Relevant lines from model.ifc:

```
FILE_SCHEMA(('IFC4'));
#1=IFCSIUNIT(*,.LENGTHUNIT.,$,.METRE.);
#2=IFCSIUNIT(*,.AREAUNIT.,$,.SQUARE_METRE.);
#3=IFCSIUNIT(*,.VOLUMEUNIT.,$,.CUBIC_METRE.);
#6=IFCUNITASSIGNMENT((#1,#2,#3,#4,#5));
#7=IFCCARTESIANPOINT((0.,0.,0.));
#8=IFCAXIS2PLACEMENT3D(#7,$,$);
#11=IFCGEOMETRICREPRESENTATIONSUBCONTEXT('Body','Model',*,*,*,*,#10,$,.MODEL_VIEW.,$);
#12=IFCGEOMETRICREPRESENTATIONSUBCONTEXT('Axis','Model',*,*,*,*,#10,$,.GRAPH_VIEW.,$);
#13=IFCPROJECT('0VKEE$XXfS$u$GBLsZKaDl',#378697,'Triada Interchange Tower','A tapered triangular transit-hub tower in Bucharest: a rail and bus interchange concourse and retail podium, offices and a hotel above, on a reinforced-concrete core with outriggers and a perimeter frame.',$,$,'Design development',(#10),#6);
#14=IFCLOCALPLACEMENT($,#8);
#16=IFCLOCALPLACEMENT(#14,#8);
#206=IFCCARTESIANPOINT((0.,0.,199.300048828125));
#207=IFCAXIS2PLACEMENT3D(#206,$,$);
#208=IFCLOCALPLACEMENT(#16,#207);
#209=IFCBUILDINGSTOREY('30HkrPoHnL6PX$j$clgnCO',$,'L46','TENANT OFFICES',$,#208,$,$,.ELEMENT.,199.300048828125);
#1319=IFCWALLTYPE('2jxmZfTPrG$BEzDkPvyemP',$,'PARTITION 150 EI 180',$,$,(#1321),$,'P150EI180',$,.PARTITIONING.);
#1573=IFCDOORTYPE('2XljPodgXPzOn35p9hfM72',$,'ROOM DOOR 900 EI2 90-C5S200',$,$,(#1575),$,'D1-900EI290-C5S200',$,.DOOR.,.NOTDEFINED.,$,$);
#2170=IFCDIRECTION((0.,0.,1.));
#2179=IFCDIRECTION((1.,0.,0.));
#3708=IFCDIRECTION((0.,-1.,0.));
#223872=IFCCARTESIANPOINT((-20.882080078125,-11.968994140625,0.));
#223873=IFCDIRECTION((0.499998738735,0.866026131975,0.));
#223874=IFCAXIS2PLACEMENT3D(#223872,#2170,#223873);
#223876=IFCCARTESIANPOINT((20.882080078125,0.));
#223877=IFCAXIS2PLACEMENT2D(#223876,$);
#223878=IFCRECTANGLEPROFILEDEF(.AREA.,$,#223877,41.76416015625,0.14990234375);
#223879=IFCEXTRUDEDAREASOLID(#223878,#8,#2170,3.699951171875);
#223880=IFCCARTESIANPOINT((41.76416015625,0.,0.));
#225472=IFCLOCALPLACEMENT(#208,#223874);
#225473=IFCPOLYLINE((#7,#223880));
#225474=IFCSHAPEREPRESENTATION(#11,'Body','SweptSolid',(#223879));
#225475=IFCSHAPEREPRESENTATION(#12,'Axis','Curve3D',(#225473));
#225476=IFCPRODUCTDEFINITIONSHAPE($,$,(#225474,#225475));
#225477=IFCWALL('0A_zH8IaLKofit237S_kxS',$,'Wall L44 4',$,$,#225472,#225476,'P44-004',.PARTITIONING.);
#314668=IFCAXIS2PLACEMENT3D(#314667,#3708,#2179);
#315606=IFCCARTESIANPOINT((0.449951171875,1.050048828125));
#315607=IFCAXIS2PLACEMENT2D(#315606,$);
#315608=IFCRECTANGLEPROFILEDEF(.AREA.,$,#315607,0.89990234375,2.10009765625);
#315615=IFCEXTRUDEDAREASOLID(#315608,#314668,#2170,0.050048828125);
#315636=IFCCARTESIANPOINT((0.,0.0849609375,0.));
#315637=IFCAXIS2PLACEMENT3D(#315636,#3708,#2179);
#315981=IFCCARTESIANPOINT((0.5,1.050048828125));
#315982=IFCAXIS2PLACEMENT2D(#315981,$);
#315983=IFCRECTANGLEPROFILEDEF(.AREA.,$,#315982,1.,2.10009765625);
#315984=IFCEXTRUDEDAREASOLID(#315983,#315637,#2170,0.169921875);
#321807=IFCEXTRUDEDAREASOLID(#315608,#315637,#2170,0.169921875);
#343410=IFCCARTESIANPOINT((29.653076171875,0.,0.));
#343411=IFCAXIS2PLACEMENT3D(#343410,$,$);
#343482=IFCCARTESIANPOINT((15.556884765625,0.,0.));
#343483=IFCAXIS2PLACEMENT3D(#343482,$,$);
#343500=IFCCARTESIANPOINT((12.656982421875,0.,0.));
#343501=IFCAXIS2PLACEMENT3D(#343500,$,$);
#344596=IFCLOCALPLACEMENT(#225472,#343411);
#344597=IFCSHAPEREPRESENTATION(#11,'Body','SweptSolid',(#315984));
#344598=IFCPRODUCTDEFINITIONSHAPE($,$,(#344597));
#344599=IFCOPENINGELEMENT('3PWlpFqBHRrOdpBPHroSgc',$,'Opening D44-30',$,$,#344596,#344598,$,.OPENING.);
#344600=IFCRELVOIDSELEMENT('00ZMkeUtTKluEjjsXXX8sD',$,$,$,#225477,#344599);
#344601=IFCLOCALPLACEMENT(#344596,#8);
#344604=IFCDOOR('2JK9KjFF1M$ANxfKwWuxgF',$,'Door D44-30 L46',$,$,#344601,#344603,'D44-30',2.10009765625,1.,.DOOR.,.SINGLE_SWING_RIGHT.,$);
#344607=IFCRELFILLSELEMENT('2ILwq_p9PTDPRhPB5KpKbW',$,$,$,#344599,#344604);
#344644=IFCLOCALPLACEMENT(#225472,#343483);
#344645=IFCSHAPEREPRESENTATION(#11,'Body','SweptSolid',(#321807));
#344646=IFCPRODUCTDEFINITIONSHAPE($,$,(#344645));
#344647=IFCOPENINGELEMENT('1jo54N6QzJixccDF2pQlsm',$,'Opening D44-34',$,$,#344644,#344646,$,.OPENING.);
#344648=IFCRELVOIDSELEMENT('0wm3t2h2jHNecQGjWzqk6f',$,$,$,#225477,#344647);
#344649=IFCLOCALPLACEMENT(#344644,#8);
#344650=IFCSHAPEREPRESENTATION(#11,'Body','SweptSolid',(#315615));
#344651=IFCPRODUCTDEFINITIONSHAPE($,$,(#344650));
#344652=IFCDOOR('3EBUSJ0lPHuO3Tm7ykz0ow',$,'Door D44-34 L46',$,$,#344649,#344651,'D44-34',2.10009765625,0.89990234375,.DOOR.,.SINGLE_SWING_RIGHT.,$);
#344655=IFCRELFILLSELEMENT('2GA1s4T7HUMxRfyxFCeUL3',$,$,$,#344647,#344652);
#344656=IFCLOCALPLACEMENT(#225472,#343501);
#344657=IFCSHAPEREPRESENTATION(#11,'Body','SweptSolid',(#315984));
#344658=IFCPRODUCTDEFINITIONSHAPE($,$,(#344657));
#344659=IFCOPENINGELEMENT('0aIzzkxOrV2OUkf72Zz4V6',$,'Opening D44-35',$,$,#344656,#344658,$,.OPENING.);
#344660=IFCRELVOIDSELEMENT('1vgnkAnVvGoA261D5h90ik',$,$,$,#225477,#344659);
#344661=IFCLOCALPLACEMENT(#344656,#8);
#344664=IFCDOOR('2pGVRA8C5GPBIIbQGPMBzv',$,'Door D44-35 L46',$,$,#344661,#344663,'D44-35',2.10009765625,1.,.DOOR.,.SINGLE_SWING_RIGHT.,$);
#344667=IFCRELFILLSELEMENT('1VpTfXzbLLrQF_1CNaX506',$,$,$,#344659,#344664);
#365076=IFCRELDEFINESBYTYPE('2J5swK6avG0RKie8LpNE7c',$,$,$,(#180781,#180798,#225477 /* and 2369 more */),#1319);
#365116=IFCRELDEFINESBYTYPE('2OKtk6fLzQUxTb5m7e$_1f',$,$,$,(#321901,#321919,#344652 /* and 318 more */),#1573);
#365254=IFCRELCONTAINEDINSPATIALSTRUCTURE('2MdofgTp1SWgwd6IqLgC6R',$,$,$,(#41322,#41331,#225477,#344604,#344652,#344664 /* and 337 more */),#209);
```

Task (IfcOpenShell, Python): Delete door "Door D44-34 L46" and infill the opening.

```python
import ifcopenshell
import ifcopenshell.api.feature
import ifcopenshell.api.root
import ifcopenshell.geom
import ifcopenshell.util.shape

model = ifcopenshell.open("model.ifc")
settings = ifcopenshell.geom.settings()


def volume(element):
    """Net volume in cubic metres, openings subtracted."""
    shape = ifcopenshell.geom.create_shape(settings, element)
    return ifcopenshell.util.shape.get_volume(shape.geometry)


door = model.by_guid("3EBUSJ0lPHuO3Tm7ykz0ow")
opening = door.FillsVoids[0].RelatingOpeningElement
wall = opening.VoidsElements[0].RelatingBuildingElement
before = volume(wall)

ifcopenshell.api.root.remove_product(model, product=door)
ifcopenshell.api.feature.remove_feature(model, feature=opening)

after = volume(wall)

print(f"wall volume {before:.3f} -> {after:.3f} m3")

model.write("model-out.ifc")
```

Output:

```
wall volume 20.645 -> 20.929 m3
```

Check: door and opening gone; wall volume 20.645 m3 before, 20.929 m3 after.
